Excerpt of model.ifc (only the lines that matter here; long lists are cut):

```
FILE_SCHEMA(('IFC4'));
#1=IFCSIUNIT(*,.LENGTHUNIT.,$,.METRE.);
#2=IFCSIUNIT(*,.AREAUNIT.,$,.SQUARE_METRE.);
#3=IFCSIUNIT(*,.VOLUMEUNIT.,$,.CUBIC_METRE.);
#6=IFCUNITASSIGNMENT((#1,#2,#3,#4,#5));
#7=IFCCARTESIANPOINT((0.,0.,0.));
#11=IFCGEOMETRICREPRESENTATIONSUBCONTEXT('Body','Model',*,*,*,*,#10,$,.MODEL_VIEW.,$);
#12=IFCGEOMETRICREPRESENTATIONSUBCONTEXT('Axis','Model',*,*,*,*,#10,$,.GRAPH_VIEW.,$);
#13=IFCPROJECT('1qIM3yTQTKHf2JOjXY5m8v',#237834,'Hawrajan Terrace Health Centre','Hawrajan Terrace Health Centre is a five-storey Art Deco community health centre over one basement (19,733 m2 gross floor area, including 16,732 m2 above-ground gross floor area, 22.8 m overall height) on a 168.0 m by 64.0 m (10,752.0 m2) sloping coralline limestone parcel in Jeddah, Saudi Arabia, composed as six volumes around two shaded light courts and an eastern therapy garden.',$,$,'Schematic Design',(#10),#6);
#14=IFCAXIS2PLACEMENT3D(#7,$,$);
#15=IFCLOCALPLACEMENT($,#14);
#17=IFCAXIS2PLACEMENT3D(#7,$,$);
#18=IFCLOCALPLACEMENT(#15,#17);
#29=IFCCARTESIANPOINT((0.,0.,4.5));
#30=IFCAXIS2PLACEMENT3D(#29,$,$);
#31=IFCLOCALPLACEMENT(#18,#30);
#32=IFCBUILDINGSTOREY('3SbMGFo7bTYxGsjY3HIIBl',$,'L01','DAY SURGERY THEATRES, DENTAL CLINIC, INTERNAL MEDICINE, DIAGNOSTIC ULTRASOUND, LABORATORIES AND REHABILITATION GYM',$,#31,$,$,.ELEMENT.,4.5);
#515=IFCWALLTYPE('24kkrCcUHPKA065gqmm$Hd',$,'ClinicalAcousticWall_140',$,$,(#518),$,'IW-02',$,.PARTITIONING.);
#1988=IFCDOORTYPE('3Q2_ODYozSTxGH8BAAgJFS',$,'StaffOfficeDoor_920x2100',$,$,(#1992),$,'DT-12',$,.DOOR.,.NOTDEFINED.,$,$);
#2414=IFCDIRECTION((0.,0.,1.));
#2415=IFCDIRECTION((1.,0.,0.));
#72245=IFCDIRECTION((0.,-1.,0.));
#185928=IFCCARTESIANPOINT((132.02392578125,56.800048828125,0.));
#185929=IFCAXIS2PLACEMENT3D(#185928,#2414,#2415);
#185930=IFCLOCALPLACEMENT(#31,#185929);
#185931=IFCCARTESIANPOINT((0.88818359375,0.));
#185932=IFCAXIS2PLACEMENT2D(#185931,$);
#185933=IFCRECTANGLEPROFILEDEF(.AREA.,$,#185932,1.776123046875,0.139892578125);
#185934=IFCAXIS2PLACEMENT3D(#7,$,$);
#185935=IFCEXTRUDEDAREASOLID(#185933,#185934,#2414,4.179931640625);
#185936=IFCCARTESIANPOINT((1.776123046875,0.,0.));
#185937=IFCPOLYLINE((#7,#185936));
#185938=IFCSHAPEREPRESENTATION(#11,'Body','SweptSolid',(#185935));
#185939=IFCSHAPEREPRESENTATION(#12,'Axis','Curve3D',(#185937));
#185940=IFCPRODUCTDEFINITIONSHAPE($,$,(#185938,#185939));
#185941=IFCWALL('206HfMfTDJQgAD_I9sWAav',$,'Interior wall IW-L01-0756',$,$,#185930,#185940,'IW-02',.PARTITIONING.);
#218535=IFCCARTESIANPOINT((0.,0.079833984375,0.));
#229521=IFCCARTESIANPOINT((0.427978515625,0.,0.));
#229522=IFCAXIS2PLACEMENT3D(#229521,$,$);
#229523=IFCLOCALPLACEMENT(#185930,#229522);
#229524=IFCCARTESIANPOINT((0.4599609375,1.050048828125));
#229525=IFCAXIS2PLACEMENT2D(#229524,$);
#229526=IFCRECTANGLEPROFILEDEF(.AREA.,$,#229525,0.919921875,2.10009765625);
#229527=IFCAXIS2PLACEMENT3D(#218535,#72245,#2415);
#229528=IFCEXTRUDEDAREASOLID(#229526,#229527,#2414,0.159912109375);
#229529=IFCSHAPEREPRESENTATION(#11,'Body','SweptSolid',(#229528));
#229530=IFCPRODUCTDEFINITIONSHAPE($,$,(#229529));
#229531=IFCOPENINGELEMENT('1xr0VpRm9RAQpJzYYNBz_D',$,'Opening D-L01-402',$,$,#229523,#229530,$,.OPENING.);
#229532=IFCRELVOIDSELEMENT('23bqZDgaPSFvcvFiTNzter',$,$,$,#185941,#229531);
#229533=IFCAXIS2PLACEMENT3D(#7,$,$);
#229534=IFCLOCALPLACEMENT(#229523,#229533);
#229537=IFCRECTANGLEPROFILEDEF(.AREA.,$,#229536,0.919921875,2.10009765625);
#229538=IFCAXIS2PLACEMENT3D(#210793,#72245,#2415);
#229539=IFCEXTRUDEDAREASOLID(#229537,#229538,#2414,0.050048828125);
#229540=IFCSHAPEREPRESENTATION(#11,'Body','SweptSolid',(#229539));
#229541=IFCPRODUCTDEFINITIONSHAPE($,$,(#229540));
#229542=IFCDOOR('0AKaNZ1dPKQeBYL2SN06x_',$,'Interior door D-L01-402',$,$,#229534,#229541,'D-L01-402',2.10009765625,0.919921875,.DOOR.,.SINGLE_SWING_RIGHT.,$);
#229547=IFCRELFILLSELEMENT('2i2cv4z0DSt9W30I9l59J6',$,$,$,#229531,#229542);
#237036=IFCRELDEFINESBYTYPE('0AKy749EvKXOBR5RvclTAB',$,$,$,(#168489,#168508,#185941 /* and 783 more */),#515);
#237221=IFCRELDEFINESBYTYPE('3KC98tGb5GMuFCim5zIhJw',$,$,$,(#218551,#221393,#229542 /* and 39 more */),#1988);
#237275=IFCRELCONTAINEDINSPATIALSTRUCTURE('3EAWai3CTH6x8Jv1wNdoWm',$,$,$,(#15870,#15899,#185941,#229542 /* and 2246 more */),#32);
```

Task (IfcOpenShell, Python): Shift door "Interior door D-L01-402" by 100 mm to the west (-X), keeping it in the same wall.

```python
import ifcopenshell
import ifcopenshell.api.geometry
import ifcopenshell.util.placement
import ifcopenshell.util.unit

model = ifcopenshell.open("model.ifc")
unit_scale = ifcopenshell.util.unit.calculate_unit_scale(model)

door = model.by_id(229542)
opening = door.FillsVoids[0].RelatingOpeningElement
wall = opening.VoidsElements[0].RelatingBuildingElement

wall_matrix = ifcopenshell.util.placement.get_local_placement(wall.ObjectPlacement)
shift = wall_matrix[:3, 0] * -0.1 / unit_scale
before = ifcopenshell.util.placement.get_local_placement(door.ObjectPlacement)[:3, 3].copy()

# The door is placed relative to its opening, so it follows when the opening moves.
matrix = ifcopenshell.util.placement.get_local_placement(opening.ObjectPlacement)
matrix[:3, 3] += shift
ifcopenshell.api.geometry.edit_object_placement(
    model, product=opening, matrix=matrix, is_si=False, should_transform_children=True
)

after = ifcopenshell.util.placement.get_local_placement(door.ObjectPlacement)[:3, 3]
print("door moved by", (after - before).round(3) + 0.0)

model.write("model_v2.ifc")
```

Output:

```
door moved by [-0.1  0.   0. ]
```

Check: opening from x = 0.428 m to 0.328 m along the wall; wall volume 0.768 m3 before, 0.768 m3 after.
